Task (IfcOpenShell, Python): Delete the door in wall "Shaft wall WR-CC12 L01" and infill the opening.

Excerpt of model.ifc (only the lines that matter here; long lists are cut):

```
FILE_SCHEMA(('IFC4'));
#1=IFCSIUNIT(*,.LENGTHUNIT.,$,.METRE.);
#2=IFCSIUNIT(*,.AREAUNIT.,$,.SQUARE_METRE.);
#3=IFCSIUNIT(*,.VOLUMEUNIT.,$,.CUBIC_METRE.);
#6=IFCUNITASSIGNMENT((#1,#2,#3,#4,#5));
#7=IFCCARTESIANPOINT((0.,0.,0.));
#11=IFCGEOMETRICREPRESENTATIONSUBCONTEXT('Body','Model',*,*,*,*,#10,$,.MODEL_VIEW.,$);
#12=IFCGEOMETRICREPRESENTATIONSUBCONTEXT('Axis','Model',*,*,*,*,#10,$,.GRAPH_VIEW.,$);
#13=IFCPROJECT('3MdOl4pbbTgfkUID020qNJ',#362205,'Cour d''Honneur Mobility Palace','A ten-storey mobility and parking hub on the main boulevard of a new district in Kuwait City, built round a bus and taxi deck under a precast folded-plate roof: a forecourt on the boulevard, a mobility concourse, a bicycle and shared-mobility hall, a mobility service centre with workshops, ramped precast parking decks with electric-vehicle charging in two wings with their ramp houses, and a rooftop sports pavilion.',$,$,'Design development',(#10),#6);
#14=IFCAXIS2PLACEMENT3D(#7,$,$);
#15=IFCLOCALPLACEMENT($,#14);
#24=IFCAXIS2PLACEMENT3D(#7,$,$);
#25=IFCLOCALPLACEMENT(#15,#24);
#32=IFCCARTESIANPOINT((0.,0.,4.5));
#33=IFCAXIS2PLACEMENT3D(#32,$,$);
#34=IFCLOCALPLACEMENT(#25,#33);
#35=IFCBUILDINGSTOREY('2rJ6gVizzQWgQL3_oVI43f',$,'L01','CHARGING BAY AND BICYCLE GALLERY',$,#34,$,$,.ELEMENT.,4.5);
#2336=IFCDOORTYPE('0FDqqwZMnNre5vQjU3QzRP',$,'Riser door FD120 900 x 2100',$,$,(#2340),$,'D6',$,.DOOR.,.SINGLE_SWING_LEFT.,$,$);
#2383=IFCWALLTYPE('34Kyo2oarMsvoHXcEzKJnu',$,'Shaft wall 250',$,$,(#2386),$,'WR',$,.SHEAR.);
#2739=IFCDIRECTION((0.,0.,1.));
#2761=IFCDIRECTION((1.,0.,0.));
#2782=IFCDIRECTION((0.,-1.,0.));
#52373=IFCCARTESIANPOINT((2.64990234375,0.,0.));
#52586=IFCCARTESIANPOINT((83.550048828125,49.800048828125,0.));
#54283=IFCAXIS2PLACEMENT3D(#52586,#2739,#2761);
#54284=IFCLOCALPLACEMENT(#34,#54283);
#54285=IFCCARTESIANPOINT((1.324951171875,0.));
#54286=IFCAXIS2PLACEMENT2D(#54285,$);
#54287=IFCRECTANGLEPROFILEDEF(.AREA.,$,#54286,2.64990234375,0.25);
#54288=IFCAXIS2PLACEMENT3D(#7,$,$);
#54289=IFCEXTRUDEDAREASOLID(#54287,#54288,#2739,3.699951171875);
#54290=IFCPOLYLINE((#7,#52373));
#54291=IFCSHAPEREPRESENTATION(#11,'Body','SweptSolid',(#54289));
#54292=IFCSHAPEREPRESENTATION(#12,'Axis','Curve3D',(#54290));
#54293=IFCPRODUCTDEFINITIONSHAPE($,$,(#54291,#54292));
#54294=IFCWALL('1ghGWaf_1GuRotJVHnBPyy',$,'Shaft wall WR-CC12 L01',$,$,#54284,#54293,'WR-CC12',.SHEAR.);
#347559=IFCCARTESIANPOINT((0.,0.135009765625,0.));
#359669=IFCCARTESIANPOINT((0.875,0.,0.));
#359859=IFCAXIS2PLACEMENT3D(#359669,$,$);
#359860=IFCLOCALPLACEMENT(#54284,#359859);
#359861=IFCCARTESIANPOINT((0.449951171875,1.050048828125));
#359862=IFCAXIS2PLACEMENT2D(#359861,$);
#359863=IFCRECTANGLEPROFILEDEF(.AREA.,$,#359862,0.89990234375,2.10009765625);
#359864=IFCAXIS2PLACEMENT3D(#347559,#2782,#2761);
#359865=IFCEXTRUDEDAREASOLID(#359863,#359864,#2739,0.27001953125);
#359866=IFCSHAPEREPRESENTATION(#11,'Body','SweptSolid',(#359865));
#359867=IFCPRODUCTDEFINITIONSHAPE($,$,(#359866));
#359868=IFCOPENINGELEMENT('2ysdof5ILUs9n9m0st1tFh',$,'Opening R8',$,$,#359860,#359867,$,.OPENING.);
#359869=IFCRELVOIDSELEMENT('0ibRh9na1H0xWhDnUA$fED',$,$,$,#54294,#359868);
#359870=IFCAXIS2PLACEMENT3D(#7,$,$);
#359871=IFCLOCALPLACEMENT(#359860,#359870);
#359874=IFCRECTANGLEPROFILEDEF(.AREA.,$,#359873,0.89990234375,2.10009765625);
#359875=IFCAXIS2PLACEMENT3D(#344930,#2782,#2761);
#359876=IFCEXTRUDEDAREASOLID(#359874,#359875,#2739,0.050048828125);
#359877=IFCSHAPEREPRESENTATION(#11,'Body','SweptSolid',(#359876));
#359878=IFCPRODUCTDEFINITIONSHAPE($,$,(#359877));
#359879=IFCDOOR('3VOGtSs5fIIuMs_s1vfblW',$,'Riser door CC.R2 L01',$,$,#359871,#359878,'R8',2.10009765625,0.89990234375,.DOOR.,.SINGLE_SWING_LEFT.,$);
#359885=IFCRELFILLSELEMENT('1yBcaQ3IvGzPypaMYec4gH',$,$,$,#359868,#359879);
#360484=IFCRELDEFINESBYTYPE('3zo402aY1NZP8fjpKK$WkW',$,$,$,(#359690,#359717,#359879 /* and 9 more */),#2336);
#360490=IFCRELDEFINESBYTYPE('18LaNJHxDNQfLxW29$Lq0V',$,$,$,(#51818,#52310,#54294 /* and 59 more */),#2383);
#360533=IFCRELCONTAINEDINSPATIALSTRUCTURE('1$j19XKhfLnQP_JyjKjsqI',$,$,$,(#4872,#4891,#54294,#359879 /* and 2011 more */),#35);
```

```python
import ifcopenshell
import ifcopenshell.api.feature
import ifcopenshell.api.root
import ifcopenshell.geom
import ifcopenshell.util.shape

model = ifcopenshell.open("model.ifc")
settings = ifcopenshell.geom.settings()


def volume(element):
    """Net volume in cubic metres, openings subtracted."""
    shape = ifcopenshell.geom.create_shape(settings, element)
    return ifcopenshell.util.shape.get_volume(shape.geometry)


door = model.by_guid("3VOGtSs5fIIuMs_s1vfblW")
opening = door.FillsVoids[0].RelatingOpeningElement
wall = opening.VoidsElements[0].RelatingBuildingElement
before = volume(wall)

ifcopenshell.api.root.remove_product(model, product=door)
ifcopenshell.api.feature.remove_feature(model, feature=opening)

after = volume(wall)

print(f"wall volume {before:.3f} -> {after:.3f} m3")

model.write("model_rev.ifc")
```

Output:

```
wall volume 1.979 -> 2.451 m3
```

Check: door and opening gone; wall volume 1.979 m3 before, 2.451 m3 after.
